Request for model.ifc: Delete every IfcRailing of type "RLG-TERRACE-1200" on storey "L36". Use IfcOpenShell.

First a look at what the model holds.

```python
import ifcopenshell
import ifcopenshell.util.element

model = ifcopenshell.open("model.ifc")
print(model.schema)
storey = next(s for s in model.by_type("IfcBuildingStorey") if s.Name == "L36")
railings = [e for e in ifcopenshell.util.element.get_decomposition(storey) if e.is_a("IfcRailing")]
seen = {}
for e in railings:
    element_type = ifcopenshell.util.element.get_type(e)
    name = element_type.Name if element_type not in (None, e) else None
    seen[name] = seen.get(name, 0) + 1
for name, count in sorted(seen.items(), key=str):
    print(count, "x", name)
```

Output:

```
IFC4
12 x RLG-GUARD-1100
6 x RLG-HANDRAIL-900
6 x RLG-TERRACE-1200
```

```python
import ifcopenshell
import ifcopenshell.api.root
import ifcopenshell.util.element

model = ifcopenshell.open("model.ifc")

storey = next(s for s in model.by_type("IfcBuildingStorey") if s.Name == "L36")
railings = [e for e in ifcopenshell.util.element.get_decomposition(storey) if e.is_a("IfcRailing")]
targets = [e for e in railings if (t := ifcopenshell.util.element.get_type(e)) not in (None, e) and t.Name == "RLG-TERRACE-1200"]

for e in targets:
    ifcopenshell.api.root.remove_product(model, product=e)
print(len(targets), "removed")

model.write("model_updated.ifc")
```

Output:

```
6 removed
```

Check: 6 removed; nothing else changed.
